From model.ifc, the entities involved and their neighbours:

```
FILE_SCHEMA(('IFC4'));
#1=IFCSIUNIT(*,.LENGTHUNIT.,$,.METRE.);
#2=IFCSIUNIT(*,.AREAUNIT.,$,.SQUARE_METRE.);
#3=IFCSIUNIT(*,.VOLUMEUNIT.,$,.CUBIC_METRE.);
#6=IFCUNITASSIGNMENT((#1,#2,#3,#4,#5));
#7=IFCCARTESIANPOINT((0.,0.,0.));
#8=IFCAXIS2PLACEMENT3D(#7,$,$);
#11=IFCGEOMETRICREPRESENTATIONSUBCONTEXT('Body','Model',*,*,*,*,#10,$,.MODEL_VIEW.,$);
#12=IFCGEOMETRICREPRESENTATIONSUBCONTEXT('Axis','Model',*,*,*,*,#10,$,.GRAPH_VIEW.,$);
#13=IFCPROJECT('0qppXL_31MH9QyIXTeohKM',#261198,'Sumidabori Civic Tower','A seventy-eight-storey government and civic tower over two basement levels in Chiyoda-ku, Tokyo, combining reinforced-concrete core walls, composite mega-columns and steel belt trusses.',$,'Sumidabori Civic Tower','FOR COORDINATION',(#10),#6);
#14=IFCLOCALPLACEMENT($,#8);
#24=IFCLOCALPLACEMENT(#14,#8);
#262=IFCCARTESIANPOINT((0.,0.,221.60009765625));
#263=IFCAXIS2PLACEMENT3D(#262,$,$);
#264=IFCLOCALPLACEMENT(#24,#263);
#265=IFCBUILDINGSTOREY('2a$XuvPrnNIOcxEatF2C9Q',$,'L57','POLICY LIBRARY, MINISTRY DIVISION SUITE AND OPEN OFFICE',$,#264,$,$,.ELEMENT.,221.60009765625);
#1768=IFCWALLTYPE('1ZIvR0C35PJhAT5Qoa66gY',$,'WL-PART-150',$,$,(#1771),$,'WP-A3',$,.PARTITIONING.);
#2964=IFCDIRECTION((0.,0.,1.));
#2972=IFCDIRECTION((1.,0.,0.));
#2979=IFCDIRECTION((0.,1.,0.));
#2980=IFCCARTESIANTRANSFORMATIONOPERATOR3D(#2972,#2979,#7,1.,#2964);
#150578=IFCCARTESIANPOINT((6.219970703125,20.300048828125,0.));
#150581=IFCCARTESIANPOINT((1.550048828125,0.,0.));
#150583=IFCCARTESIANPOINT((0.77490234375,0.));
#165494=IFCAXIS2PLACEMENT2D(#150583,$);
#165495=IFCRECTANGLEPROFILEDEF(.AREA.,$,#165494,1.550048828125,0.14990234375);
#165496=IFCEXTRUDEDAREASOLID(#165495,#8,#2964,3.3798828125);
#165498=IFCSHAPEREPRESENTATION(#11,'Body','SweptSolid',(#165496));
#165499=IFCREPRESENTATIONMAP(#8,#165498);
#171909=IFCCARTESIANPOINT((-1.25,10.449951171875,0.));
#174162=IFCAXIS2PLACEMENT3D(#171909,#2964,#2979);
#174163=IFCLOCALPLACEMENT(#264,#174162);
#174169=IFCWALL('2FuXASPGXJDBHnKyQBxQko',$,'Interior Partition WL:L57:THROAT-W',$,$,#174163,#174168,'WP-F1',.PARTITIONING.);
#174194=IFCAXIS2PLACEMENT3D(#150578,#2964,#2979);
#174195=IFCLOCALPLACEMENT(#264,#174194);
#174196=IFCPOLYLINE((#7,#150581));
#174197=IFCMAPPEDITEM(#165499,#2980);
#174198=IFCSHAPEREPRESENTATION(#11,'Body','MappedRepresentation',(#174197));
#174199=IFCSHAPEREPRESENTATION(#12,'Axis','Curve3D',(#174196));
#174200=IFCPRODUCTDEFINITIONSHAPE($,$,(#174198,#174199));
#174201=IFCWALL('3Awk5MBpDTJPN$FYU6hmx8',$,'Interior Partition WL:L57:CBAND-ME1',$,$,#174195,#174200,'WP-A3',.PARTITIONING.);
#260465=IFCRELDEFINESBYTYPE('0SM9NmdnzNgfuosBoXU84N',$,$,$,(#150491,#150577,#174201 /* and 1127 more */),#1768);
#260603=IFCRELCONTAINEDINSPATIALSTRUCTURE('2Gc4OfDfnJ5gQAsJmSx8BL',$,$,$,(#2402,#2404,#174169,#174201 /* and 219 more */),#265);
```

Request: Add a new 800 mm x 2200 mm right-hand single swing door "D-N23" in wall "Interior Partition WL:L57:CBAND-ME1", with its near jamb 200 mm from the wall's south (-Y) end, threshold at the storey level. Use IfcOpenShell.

```python
import numpy as np
import ifcopenshell
import ifcopenshell.api.feature
import ifcopenshell.api.geometry
import ifcopenshell.api.root
import ifcopenshell.api.spatial
import ifcopenshell.geom
import ifcopenshell.util.element
import ifcopenshell.util.placement
import ifcopenshell.util.representation
import ifcopenshell.util.shape
import ifcopenshell.util.unit

model = ifcopenshell.open("model.ifc")
unit_scale = ifcopenshell.util.unit.calculate_unit_scale(model)
settings = ifcopenshell.geom.settings()


def volume(element):
    """Net volume in cubic metres, openings subtracted."""
    shape = ifcopenshell.geom.create_shape(settings, element)
    return ifcopenshell.util.shape.get_volume(shape.geometry)


wall = model.by_guid("3Awk5MBpDTJPN$FYU6hmx8")
storey = ifcopenshell.util.element.get_container(wall, ifc_class="IfcBuildingStorey")
context = ifcopenshell.util.representation.get_context(model, "Model", "Body", "MODEL_VIEW")
before = volume(wall)

width, height, from_end, sill = 0.8, 2.2, 0.2, 0.0  # metres

# The wall runs along its own X axis, and the end named is its -X end.
wall_shape = ifcopenshell.geom.create_shape(settings, wall)
x, y, z = ifcopenshell.util.shape.get_vertices(wall_shape.geometry).T
start = x.min() + from_end
face, thickness = float(y.min()), float(y.max() - y.min())
wall_matrix = ifcopenshell.util.placement.get_local_placement(wall.ObjectPlacement)
level = ifcopenshell.util.placement.get_local_placement(storey.ObjectPlacement)[2, 3]


def in_wall(x, y):
    """Placement at x, y metres in the wall's axes, at sill height."""
    matrix = wall_matrix.copy()
    matrix[:, 3] = wall_matrix @ np.array([x / unit_scale, y / unit_scale, 0.0, 1.0])
    matrix[2, 3] = level + sill / unit_scale
    return matrix


# Opening: a box that overshoots both wall faces by 50 mm.
opening = ifcopenshell.api.root.create_entity(model, ifc_class="IfcOpeningElement", predefined_type="OPENING")
box = ifcopenshell.api.geometry.add_wall_representation(
    model, context=context, length=width, height=height, thickness=thickness + 0.1
)
ifcopenshell.api.geometry.assign_representation(model, product=opening, representation=box)
ifcopenshell.api.geometry.edit_object_placement(model, product=opening, matrix=in_wall(start, face - 0.05), is_si=False)
ifcopenshell.api.feature.add_feature(model, feature=opening, element=wall)

door = ifcopenshell.api.root.create_entity(model, ifc_class="IfcDoor", name="D-N23", predefined_type="DOOR")
door.OverallWidth, door.OverallHeight = width / unit_scale, height / unit_scale
door.OperationType = "SINGLE_SWING_RIGHT"
body = ifcopenshell.api.geometry.add_door_representation(
    model,
    context=context,
    overall_width=door.OverallWidth,
    overall_height=door.OverallHeight,
    operation_type="SINGLE_SWING_RIGHT",
    lining_properties={"LiningDepth": thickness / unit_scale, "ThresholdDepth": thickness / unit_scale},
)
ifcopenshell.api.geometry.assign_representation(model, product=door, representation=body)
ifcopenshell.api.spatial.assign_container(model, products=[door], relating_structure=storey)
ifcopenshell.api.feature.add_filling(model, opening=opening, element=door)

# The lining spans the wall, so the door starts at the wall face.
ifcopenshell.api.geometry.edit_object_placement(model, product=door, matrix=in_wall(start, face), is_si=False)

after = volume(wall)

print(f"wall volume {before:.3f} -> {after:.3f} m3")

model.write("model_rev.ifc")
```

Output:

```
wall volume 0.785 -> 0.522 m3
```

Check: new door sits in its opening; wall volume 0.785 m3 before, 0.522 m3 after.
